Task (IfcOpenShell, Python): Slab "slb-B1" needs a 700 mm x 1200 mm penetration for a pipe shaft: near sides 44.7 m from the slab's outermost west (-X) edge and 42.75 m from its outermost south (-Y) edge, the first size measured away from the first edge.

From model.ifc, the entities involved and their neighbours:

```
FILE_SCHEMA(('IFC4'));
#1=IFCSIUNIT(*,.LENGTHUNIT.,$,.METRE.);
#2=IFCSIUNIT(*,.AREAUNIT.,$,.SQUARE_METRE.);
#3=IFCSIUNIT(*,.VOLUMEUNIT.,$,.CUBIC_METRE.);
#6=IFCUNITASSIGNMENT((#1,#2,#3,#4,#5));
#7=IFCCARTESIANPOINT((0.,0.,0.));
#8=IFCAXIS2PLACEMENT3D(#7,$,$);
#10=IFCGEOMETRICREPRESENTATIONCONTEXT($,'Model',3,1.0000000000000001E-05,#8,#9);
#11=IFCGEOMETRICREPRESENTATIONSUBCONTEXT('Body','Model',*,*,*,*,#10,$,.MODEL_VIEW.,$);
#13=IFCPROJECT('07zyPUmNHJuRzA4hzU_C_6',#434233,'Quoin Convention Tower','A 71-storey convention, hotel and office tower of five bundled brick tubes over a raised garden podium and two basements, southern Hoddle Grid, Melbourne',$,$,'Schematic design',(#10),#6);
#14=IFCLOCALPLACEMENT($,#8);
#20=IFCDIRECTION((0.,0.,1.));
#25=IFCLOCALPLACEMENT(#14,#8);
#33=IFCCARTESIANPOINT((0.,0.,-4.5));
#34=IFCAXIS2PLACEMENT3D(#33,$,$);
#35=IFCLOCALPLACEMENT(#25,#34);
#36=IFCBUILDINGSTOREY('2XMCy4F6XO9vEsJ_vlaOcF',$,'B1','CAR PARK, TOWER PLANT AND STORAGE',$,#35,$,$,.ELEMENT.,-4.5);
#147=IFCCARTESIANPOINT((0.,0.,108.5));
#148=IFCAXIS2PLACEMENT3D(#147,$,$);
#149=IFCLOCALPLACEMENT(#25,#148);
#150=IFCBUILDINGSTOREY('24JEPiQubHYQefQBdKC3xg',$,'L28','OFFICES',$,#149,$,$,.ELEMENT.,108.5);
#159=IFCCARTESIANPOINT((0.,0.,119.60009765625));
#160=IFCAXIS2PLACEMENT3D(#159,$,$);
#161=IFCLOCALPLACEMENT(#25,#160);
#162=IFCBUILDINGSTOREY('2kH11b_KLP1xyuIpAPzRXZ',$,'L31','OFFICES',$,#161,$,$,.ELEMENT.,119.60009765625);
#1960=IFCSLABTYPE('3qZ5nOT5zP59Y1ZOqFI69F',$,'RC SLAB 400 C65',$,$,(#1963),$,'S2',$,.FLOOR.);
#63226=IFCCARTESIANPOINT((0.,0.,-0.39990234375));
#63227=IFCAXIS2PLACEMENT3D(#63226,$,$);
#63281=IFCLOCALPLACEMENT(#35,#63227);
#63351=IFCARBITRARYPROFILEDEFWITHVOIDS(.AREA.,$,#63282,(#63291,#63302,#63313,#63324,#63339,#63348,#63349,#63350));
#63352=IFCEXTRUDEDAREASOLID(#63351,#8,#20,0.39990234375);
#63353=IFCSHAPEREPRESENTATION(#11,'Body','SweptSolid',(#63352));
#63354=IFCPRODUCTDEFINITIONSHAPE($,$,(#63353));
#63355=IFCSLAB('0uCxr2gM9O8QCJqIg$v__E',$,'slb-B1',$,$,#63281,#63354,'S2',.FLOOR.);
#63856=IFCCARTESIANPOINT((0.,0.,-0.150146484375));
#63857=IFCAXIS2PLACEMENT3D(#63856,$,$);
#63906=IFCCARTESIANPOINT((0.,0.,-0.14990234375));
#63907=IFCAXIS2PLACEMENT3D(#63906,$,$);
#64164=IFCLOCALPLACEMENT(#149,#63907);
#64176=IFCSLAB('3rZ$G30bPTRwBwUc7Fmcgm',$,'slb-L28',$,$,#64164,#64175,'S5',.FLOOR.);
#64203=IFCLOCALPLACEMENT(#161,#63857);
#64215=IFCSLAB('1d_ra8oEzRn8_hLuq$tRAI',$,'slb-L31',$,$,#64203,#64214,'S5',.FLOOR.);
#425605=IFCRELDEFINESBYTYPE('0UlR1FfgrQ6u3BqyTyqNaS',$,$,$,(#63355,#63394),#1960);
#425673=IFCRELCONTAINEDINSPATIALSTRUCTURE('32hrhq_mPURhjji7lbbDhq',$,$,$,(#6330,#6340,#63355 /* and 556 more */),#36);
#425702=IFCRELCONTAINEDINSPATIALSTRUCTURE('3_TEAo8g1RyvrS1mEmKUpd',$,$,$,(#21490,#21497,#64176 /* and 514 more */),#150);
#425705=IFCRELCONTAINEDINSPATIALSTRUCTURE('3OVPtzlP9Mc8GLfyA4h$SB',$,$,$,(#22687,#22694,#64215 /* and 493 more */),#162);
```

```python
import numpy as np
import ifcopenshell
import ifcopenshell.api.feature
import ifcopenshell.api.geometry
import ifcopenshell.api.root
import ifcopenshell.geom
import ifcopenshell.util.placement
import ifcopenshell.util.representation
import ifcopenshell.util.shape
import ifcopenshell.util.unit

model = ifcopenshell.open("model.ifc")
unit_scale = ifcopenshell.util.unit.calculate_unit_scale(model)
settings = ifcopenshell.geom.settings()


def volume(element):
    """Net volume in cubic metres, openings subtracted."""
    shape = ifcopenshell.geom.create_shape(settings, element)
    return ifcopenshell.util.shape.get_volume(shape.geometry)


slab = model.by_guid("0uCxr2gM9O8QCJqIg$v__E")
before = volume(slab)

# Extent in the slab's own axes, in metres. The edges named are its -X and -Y sides.
slab_shape = ifcopenshell.geom.create_shape(settings, slab)
vertices = ifcopenshell.util.shape.get_vertices(slab_shape.geometry)
x_min, y_min, bottom = vertices.min(axis=0)
top = vertices[:, 2].max()

opening = ifcopenshell.api.root.create_entity(model, ifc_class="IfcOpeningElement", name="Pipe shaft opening", predefined_type="OPENING")
context = ifcopenshell.util.representation.get_context(model, "Model", "Body", "MODEL_VIEW")
width, depth = 0.7, 1.2
outline = [(0.0, 0.0), (width, 0.0), (width, depth), (0.0, depth), (0.0, 0.0)]
# Overshoot both faces by 50 mm so the cut is clean.
shape = ifcopenshell.api.geometry.add_slab_representation(
    model, context=context, depth=top - bottom + 0.1, polyline=outline
)
ifcopenshell.api.geometry.assign_representation(model, product=opening, representation=shape)

matrix = ifcopenshell.util.placement.get_local_placement(slab.ObjectPlacement)
matrix[:, 3] = matrix @ np.append(np.array([x_min + 44.7, y_min + 42.75, bottom - 0.05]) / unit_scale, 1.0)
ifcopenshell.api.geometry.edit_object_placement(model, product=opening, matrix=matrix, is_si=False)
ifcopenshell.api.feature.add_feature(model, feature=opening, element=slab)

after = volume(slab)

print(f"slab volume {before:.3f} -> {after:.3f} m3")

model.write("model-out.ifc")
```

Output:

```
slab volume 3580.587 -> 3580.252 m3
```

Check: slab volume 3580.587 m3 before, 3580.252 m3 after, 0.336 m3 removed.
